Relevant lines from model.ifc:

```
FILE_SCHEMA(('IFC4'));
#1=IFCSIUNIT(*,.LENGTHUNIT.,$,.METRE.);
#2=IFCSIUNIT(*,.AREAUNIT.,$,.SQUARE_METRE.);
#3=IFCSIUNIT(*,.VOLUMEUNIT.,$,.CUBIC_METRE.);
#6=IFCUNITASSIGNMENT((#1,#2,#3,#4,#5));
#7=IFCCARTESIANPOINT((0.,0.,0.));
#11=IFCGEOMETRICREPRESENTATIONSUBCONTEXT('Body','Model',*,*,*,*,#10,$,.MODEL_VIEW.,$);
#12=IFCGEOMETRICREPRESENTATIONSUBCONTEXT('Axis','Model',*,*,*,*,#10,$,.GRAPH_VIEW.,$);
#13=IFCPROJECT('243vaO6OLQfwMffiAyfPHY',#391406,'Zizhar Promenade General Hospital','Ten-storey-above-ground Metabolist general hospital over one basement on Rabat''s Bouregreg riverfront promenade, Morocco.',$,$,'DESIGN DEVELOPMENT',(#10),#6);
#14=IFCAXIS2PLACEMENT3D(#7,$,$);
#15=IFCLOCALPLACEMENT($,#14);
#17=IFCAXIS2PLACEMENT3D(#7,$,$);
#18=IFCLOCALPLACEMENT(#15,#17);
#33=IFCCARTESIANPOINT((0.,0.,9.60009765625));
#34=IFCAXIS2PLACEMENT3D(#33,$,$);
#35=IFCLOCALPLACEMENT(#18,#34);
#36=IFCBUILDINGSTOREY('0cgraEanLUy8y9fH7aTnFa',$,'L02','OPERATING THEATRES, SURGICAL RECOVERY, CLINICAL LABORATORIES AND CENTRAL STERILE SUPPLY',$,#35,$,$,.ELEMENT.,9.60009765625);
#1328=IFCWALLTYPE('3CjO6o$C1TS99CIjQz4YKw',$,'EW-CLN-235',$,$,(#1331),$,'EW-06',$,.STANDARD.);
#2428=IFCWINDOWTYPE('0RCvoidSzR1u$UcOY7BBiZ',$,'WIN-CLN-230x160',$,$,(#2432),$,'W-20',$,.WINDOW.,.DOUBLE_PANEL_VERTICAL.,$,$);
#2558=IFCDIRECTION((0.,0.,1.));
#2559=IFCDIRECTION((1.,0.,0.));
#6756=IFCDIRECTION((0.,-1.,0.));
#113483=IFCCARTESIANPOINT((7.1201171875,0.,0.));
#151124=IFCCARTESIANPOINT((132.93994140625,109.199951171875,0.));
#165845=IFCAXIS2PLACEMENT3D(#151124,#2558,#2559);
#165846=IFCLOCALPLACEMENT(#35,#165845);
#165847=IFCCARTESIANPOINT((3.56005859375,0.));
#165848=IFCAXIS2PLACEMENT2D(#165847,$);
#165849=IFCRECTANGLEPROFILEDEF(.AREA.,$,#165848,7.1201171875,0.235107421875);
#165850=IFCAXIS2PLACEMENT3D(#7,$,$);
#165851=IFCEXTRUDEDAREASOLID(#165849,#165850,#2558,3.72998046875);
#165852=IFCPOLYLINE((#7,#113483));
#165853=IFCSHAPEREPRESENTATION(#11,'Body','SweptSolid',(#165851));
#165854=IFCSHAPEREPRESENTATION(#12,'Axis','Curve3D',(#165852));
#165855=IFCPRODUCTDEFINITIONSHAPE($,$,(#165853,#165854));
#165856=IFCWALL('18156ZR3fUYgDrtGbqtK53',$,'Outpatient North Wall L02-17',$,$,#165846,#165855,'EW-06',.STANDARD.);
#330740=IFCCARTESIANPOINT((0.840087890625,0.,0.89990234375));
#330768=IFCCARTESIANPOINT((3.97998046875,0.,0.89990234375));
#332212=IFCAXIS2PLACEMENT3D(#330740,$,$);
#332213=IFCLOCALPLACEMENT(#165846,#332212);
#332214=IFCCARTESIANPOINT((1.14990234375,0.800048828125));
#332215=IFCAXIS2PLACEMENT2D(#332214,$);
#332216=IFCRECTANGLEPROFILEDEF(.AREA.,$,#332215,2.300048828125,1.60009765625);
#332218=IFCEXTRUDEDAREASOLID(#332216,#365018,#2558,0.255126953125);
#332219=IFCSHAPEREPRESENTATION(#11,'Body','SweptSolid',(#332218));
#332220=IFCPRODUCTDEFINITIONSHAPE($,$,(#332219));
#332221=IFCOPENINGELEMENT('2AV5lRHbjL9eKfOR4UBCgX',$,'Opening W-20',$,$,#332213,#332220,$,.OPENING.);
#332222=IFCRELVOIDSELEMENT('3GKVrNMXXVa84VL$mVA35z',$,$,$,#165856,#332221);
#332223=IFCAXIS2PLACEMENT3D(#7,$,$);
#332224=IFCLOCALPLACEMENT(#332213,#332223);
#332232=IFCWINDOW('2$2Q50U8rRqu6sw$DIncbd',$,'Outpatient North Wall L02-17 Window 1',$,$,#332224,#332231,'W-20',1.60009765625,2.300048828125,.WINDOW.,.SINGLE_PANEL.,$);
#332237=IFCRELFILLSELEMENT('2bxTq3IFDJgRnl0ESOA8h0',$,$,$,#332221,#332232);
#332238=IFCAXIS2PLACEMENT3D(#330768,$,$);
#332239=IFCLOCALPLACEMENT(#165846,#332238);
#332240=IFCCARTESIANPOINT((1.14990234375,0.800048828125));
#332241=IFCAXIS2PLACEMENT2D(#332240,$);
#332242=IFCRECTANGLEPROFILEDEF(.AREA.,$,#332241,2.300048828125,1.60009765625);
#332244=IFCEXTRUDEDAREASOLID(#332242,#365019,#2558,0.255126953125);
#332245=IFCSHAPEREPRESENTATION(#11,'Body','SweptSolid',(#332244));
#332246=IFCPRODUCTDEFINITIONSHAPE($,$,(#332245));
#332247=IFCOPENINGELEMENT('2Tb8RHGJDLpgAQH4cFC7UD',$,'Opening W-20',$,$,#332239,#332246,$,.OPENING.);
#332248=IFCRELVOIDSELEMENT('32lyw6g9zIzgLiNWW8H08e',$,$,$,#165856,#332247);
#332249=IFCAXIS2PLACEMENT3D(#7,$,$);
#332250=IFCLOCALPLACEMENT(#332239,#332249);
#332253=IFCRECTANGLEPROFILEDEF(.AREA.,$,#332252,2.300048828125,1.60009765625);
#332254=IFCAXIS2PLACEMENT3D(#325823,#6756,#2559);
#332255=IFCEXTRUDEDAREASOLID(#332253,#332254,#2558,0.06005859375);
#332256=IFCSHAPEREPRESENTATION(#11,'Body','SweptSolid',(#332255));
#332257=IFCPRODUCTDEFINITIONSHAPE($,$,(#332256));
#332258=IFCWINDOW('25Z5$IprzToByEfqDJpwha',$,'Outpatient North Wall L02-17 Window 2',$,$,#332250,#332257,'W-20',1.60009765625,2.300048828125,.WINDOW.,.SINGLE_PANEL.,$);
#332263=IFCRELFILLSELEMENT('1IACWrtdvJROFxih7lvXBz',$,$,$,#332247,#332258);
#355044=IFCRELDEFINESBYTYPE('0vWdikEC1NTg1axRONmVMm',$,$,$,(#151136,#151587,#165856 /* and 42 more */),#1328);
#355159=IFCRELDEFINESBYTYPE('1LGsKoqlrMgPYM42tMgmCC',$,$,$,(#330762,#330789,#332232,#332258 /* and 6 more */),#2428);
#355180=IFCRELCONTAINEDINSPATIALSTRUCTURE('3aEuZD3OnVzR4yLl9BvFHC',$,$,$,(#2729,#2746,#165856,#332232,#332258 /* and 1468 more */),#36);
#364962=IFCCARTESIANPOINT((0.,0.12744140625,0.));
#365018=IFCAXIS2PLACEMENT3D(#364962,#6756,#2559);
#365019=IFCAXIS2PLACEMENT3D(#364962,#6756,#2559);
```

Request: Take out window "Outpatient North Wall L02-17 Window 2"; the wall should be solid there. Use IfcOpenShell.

```python
import ifcopenshell
import ifcopenshell.api.feature
import ifcopenshell.api.root
import ifcopenshell.geom
import ifcopenshell.util.shape

model = ifcopenshell.open("model.ifc")
settings = ifcopenshell.geom.settings()


def volume(element):
    """Net volume in cubic metres, openings subtracted."""
    shape = ifcopenshell.geom.create_shape(settings, element)
    return ifcopenshell.util.shape.get_volume(shape.geometry)


window = model.by_guid("25Z5$IprzToByEfqDJpwha")
opening = window.FillsVoids[0].RelatingOpeningElement
wall = opening.VoidsElements[0].RelatingBuildingElement
before = volume(wall)

ifcopenshell.api.root.remove_product(model, product=window)
ifcopenshell.api.feature.remove_feature(model, feature=opening)

after = volume(wall)

print(f"wall volume {before:.3f} -> {after:.3f} m3")

model.write("model_updated.ifc")
```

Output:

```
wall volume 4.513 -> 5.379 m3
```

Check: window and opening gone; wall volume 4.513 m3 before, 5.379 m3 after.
